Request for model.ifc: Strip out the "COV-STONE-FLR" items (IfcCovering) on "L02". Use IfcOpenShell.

First a look at what the model holds.

```python
import ifcopenshell
import ifcopenshell.util.element

model = ifcopenshell.open("model.ifc")
print(model.schema)
storey = next(s for s in model.by_type("IfcBuildingStorey") if s.Name == "L02")
coverings = [e for e in ifcopenshell.util.element.get_decomposition(storey) if e.is_a("IfcCovering")]
seen = {}
for e in coverings:
    element_type = ifcopenshell.util.element.get_type(e)
    name = element_type.Name if element_type not in (None, e) else None
    seen[name] = seen.get(name, 0) + 1
for name, count in sorted(seen.items(), key=str):
    print(count, "x", name)
```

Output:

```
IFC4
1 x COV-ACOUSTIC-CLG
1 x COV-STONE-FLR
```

```python
import ifcopenshell
import ifcopenshell.api.root
import ifcopenshell.util.element

model = ifcopenshell.open("model.ifc")

storey = next(s for s in model.by_type("IfcBuildingStorey") if s.Name == "L02")
coverings = [e for e in ifcopenshell.util.element.get_decomposition(storey) if e.is_a("IfcCovering")]
targets = [e for e in coverings if (t := ifcopenshell.util.element.get_type(e)) not in (None, e) and t.Name == "COV-STONE-FLR"]

for e in targets:
    ifcopenshell.api.root.remove_product(model, product=e)
print(len(targets), "removed")

model.write("model_updated.ifc")
```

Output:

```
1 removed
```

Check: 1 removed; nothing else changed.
